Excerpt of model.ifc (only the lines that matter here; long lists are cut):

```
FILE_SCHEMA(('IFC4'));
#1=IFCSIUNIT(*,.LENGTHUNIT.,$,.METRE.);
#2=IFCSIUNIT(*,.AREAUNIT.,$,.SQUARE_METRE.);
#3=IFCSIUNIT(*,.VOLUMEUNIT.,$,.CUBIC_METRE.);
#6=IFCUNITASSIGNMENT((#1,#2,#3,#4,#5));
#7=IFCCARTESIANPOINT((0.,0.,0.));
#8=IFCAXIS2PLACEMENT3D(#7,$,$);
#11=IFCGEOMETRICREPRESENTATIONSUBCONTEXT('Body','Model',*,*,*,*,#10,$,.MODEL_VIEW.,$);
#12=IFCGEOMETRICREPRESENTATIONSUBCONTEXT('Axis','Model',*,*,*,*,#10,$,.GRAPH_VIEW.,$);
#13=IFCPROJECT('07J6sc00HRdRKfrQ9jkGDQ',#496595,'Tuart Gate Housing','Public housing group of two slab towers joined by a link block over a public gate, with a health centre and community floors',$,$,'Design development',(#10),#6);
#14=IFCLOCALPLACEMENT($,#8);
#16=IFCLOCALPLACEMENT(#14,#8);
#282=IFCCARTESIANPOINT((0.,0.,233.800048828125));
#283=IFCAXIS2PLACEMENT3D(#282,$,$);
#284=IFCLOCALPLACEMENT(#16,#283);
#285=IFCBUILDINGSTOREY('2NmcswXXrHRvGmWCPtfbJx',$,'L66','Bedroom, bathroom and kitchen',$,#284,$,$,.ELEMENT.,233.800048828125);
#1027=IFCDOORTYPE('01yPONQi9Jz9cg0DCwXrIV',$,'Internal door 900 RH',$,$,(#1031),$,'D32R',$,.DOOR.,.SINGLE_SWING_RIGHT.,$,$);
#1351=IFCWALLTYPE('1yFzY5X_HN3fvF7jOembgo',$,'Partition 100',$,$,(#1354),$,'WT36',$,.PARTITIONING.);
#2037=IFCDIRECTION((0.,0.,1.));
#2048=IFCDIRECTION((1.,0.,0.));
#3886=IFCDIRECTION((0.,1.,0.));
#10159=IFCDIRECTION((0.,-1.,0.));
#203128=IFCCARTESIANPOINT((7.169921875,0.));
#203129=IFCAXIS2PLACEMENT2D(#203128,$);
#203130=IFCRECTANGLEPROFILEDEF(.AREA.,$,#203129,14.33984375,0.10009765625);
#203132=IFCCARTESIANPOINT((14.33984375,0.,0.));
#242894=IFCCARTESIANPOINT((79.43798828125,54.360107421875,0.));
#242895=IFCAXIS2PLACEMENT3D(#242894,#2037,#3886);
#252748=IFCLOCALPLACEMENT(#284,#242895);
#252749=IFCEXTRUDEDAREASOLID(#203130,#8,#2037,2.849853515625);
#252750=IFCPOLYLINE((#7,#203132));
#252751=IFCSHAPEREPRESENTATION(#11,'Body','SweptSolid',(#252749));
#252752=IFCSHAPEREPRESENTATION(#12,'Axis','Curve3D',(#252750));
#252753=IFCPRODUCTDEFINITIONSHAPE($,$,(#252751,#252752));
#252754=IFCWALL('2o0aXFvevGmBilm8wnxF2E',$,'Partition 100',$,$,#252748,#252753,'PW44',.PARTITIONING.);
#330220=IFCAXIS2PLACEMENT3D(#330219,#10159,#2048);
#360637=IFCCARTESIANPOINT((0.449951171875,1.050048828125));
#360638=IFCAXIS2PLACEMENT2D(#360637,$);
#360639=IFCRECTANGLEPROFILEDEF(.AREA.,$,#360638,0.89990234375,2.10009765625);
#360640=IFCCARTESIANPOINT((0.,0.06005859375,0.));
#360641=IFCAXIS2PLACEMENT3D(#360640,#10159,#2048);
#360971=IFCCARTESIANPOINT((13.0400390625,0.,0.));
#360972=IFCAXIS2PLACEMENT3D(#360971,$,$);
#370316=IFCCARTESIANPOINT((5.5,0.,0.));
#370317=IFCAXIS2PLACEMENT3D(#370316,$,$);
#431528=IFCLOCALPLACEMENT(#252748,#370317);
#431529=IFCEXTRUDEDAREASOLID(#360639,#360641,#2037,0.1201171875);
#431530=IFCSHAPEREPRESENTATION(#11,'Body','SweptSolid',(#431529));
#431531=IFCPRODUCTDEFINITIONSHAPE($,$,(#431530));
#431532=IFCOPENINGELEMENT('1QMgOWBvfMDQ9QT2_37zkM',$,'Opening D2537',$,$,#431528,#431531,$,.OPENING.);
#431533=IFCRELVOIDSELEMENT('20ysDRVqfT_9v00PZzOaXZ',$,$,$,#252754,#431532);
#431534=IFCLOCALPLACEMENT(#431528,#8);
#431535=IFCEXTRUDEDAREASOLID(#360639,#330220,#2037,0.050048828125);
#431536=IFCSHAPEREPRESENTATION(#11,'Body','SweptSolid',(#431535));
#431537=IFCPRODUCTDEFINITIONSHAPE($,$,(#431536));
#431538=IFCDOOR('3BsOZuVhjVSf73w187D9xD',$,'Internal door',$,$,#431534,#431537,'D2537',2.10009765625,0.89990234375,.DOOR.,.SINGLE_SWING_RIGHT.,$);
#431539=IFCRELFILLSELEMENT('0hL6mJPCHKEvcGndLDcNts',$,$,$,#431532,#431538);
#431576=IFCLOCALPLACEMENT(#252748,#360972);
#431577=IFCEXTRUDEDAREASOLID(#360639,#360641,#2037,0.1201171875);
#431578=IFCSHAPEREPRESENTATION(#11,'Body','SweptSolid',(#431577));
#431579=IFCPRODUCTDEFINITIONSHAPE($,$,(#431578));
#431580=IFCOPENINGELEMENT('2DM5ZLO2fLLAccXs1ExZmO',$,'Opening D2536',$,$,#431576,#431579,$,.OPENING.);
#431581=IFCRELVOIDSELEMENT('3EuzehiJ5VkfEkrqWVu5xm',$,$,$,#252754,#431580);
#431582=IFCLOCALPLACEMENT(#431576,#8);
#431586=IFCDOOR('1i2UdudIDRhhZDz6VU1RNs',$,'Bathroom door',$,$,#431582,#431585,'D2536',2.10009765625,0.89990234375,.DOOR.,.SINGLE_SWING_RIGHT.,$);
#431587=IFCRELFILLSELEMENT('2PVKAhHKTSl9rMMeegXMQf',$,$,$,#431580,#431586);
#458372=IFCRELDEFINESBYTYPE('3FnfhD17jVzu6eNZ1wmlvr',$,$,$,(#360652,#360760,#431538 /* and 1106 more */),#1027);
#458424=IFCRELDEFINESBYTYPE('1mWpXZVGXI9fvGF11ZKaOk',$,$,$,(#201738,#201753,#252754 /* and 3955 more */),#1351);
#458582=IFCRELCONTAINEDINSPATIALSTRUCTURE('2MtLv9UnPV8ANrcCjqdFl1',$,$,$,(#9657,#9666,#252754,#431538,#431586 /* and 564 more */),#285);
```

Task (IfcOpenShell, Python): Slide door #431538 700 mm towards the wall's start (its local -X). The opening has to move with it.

```python
import ifcopenshell
import ifcopenshell.api.geometry
import ifcopenshell.util.placement

model = ifcopenshell.open("model.ifc")

door = model.by_guid("3BsOZuVhjVSf73w187D9xD")
opening = door.FillsVoids[0].RelatingOpeningElement
wall = opening.VoidsElements[0].RelatingBuildingElement

wall_matrix = ifcopenshell.util.placement.get_local_placement(wall.ObjectPlacement)
shift = wall_matrix[:3, 0] * -0.7
before = ifcopenshell.util.placement.get_local_placement(door.ObjectPlacement)[:3, 3].copy()

# The door is placed relative to its opening, so it follows when the opening moves.
matrix = ifcopenshell.util.placement.get_local_placement(opening.ObjectPlacement)
matrix[:3, 3] += shift
ifcopenshell.api.geometry.edit_object_placement(
    model, product=opening, matrix=matrix, is_si=False, should_transform_children=True
)

after = ifcopenshell.util.placement.get_local_placement(door.ObjectPlacement)[:3, 3]
print("door moved by", (after - before).round(3) + 0.0)

model.write("model_rev.ifc")
```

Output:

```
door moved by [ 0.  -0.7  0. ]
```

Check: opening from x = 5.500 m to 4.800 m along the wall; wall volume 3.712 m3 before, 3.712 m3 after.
